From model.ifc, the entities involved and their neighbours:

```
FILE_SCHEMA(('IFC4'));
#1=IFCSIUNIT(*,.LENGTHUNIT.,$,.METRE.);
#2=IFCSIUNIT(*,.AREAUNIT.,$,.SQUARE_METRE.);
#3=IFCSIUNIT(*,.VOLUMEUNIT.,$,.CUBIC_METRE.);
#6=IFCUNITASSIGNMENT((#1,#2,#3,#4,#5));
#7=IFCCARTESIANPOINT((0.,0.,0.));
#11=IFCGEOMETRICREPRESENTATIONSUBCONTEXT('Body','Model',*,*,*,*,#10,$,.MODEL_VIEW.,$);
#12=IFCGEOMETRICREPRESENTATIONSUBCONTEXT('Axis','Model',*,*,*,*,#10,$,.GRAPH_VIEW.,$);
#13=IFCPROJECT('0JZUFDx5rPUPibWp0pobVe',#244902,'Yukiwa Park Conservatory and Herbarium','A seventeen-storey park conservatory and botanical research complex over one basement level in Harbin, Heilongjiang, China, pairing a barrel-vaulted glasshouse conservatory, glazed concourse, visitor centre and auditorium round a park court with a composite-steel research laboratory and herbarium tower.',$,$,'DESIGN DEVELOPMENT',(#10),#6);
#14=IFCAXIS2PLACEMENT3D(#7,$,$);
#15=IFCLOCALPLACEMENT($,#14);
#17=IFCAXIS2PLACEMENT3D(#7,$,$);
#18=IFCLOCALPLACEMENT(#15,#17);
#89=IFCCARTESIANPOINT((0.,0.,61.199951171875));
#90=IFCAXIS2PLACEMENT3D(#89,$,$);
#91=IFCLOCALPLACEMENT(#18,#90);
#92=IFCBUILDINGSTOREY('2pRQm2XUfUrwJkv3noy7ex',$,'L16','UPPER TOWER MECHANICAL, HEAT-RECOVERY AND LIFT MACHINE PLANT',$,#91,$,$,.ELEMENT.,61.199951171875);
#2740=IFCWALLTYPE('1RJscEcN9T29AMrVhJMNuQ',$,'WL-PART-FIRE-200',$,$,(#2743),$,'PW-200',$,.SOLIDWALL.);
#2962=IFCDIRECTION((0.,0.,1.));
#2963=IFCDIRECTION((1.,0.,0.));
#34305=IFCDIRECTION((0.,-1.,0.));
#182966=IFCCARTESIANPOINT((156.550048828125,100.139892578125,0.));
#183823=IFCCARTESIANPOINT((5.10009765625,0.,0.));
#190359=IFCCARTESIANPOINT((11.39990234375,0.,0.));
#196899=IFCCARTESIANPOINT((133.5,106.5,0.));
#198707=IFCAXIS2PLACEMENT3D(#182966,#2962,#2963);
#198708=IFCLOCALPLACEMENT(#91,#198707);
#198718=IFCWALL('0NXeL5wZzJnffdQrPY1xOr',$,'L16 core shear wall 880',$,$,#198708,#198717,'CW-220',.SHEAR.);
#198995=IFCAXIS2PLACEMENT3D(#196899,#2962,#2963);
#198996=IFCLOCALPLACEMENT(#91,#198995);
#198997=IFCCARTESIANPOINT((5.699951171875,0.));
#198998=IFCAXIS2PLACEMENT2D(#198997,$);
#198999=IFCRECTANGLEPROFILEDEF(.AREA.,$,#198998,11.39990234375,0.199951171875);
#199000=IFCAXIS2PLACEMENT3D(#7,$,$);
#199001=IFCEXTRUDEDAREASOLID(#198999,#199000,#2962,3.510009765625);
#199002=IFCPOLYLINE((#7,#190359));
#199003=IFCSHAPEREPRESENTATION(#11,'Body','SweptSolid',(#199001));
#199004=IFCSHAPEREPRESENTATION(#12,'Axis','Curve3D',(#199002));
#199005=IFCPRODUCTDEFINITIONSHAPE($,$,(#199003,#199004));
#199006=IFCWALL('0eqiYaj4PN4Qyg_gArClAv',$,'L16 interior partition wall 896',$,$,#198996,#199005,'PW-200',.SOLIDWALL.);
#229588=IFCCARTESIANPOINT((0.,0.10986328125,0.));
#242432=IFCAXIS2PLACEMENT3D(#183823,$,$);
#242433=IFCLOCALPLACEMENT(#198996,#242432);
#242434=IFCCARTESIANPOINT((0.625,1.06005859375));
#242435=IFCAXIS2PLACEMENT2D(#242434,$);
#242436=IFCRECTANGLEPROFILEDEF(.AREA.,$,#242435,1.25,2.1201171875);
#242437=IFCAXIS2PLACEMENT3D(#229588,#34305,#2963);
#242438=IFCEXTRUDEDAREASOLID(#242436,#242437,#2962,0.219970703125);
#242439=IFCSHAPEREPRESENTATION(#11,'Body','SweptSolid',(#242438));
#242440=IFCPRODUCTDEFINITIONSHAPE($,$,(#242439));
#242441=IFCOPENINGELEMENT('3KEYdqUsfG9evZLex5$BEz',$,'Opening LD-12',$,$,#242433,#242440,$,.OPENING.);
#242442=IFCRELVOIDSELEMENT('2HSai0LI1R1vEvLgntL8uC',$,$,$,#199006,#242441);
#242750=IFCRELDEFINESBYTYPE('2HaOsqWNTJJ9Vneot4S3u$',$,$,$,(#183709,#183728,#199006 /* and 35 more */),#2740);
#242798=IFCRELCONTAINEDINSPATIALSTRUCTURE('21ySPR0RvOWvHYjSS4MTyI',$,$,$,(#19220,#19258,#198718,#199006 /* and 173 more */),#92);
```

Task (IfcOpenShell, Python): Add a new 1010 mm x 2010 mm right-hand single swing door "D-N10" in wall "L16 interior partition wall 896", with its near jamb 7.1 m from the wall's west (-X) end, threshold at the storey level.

```python
import numpy as np
import ifcopenshell
import ifcopenshell.api.feature
import ifcopenshell.api.geometry
import ifcopenshell.api.root
import ifcopenshell.api.spatial
import ifcopenshell.geom
import ifcopenshell.util.element
import ifcopenshell.util.placement
import ifcopenshell.util.representation
import ifcopenshell.util.shape
import ifcopenshell.util.unit

model = ifcopenshell.open("model.ifc")
unit_scale = ifcopenshell.util.unit.calculate_unit_scale(model)
settings = ifcopenshell.geom.settings()


def volume(element):
    """Net volume in cubic metres, openings subtracted."""
    shape = ifcopenshell.geom.create_shape(settings, element)
    return ifcopenshell.util.shape.get_volume(shape.geometry)


wall = model.by_guid("0eqiYaj4PN4Qyg_gArClAv")
storey = ifcopenshell.util.element.get_container(wall, ifc_class="IfcBuildingStorey")
context = ifcopenshell.util.representation.get_context(model, "Model", "Body", "MODEL_VIEW")
before = volume(wall)

width, height, from_end, sill = 1.01, 2.01, 7.1, 0.0  # metres

# The wall runs along its own X axis, and the end named is its -X end.
wall_shape = ifcopenshell.geom.create_shape(settings, wall)
x, y, z = ifcopenshell.util.shape.get_vertices(wall_shape.geometry).T
start = x.min() + from_end
face, thickness = float(y.min()), float(y.max() - y.min())
wall_matrix = ifcopenshell.util.placement.get_local_placement(wall.ObjectPlacement)
level = ifcopenshell.util.placement.get_local_placement(storey.ObjectPlacement)[2, 3]


def in_wall(x, y):
    """Placement at x, y metres in the wall's axes, at sill height."""
    matrix = wall_matrix.copy()
    matrix[:, 3] = wall_matrix @ np.array([x / unit_scale, y / unit_scale, 0.0, 1.0])
    matrix[2, 3] = level + sill / unit_scale
    return matrix


# Opening: a box that overshoots both wall faces by 50 mm.
opening = ifcopenshell.api.root.create_entity(model, ifc_class="IfcOpeningElement", predefined_type="OPENING")
box = ifcopenshell.api.geometry.add_wall_representation(
    model, context=context, length=width, height=height, thickness=thickness + 0.1
)
ifcopenshell.api.geometry.assign_representation(model, product=opening, representation=box)
ifcopenshell.api.geometry.edit_object_placement(model, product=opening, matrix=in_wall(start, face - 0.05), is_si=False)
ifcopenshell.api.feature.add_feature(model, feature=opening, element=wall)

door = ifcopenshell.api.root.create_entity(model, ifc_class="IfcDoor", name="D-N10", predefined_type="DOOR")
door.OverallWidth, door.OverallHeight = width / unit_scale, height / unit_scale
door.OperationType = "SINGLE_SWING_RIGHT"
body = ifcopenshell.api.geometry.add_door_representation(
    model,
    context=context,
    overall_width=door.OverallWidth,
    overall_height=door.OverallHeight,
    operation_type="SINGLE_SWING_RIGHT",
    lining_properties={"LiningDepth": thickness / unit_scale, "ThresholdDepth": thickness / unit_scale},
)
ifcopenshell.api.geometry.assign_representation(model, product=door, representation=body)
ifcopenshell.api.spatial.assign_container(model, products=[door], relating_structure=storey)
ifcopenshell.api.feature.add_filling(model, opening=opening, element=door)

# The lining spans the wall, so the door starts at the wall face.
ifcopenshell.api.geometry.edit_object_placement(model, product=door, matrix=in_wall(start, face), is_si=False)

after = volume(wall)

print(f"wall volume {before:.3f} -> {after:.3f} m3")

model.write("model_v2.ifc")
```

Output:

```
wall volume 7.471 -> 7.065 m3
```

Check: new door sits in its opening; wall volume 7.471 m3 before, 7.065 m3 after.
